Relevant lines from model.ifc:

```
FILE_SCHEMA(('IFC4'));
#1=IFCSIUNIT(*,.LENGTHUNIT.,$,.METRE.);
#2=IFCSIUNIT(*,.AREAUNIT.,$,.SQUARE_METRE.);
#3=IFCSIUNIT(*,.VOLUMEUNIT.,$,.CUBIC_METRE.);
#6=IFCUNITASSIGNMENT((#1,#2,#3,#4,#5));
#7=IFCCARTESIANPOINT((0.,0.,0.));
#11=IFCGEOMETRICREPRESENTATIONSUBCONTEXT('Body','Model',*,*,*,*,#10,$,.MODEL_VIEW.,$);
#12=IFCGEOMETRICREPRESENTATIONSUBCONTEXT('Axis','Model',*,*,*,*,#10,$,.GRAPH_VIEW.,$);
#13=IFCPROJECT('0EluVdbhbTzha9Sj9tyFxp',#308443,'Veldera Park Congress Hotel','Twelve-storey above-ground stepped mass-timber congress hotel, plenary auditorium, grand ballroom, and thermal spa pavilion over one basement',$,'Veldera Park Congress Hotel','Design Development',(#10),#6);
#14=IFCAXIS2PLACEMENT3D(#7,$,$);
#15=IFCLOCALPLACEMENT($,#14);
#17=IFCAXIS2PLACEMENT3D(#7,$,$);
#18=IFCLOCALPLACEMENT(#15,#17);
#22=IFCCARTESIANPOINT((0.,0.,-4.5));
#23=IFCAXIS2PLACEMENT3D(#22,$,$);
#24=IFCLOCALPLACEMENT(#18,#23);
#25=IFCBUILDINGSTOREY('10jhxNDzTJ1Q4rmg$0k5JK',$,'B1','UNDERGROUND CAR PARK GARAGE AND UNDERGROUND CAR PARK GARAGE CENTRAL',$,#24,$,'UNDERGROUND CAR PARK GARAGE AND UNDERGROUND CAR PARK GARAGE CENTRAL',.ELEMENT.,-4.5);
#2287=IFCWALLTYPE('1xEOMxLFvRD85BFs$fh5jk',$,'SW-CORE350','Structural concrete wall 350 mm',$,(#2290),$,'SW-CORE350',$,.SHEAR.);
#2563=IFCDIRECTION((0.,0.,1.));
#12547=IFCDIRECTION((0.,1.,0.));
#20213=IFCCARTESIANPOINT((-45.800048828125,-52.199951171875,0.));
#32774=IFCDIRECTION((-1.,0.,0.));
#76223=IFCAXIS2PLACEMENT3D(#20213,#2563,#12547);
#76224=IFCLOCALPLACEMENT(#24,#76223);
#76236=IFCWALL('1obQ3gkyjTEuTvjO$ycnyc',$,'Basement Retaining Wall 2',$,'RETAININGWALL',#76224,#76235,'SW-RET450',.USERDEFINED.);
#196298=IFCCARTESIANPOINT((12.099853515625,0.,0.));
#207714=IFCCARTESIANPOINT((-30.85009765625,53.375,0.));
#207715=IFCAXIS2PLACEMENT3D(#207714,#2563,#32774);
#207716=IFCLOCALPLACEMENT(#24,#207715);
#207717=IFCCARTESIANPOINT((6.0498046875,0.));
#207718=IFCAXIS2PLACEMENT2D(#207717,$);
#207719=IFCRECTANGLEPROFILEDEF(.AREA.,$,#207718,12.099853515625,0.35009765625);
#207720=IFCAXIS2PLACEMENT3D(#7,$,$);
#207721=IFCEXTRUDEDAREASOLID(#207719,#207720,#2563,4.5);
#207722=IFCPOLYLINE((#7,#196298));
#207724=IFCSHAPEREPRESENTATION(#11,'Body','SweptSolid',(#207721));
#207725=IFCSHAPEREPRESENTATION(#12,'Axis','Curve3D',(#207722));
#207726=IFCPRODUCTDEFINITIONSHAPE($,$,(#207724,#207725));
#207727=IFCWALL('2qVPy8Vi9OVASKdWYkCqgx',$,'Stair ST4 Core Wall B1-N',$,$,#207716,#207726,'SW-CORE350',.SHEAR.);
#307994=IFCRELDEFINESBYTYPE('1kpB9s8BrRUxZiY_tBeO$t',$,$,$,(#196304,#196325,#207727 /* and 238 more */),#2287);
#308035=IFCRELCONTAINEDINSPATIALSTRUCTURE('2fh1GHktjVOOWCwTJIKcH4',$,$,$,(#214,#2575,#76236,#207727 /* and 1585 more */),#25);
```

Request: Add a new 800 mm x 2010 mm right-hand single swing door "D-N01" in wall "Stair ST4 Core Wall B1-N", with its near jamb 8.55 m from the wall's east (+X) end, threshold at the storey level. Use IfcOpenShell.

```python
import numpy as np
import ifcopenshell
import ifcopenshell.api.feature
import ifcopenshell.api.geometry
import ifcopenshell.api.root
import ifcopenshell.api.spatial
import ifcopenshell.geom
import ifcopenshell.util.element
import ifcopenshell.util.placement
import ifcopenshell.util.representation
import ifcopenshell.util.shape
import ifcopenshell.util.unit

model = ifcopenshell.open("model.ifc")
unit_scale = ifcopenshell.util.unit.calculate_unit_scale(model)
settings = ifcopenshell.geom.settings()


def volume(element):
    """Net volume in cubic metres, openings subtracted."""
    shape = ifcopenshell.geom.create_shape(settings, element)
    return ifcopenshell.util.shape.get_volume(shape.geometry)


wall = model.by_guid("2qVPy8Vi9OVASKdWYkCqgx")
storey = ifcopenshell.util.element.get_container(wall, ifc_class="IfcBuildingStorey")
context = ifcopenshell.util.representation.get_context(model, "Model", "Body", "MODEL_VIEW")
before = volume(wall)

width, height, from_end, sill = 0.8, 2.01, 8.55, 0.0  # metres

# The wall runs along its own X axis, and the end named is its -X end.
wall_shape = ifcopenshell.geom.create_shape(settings, wall)
x, y, z = ifcopenshell.util.shape.get_vertices(wall_shape.geometry).T
start = x.min() + from_end
face, thickness = float(y.min()), float(y.max() - y.min())
wall_matrix = ifcopenshell.util.placement.get_local_placement(wall.ObjectPlacement)
level = ifcopenshell.util.placement.get_local_placement(storey.ObjectPlacement)[2, 3]


def in_wall(x, y):
    """Placement at x, y metres in the wall's axes, at sill height."""
    matrix = wall_matrix.copy()
    matrix[:, 3] = wall_matrix @ np.array([x / unit_scale, y / unit_scale, 0.0, 1.0])
    matrix[2, 3] = level + sill / unit_scale
    return matrix


# Opening: a box that overshoots both wall faces by 50 mm.
opening = ifcopenshell.api.root.create_entity(model, ifc_class="IfcOpeningElement", predefined_type="OPENING")
box = ifcopenshell.api.geometry.add_wall_representation(
    model, context=context, length=width, height=height, thickness=thickness + 0.1
)
ifcopenshell.api.geometry.assign_representation(model, product=opening, representation=box)
ifcopenshell.api.geometry.edit_object_placement(model, product=opening, matrix=in_wall(start, face - 0.05), is_si=False)
ifcopenshell.api.feature.add_feature(model, feature=opening, element=wall)

door = ifcopenshell.api.root.create_entity(model, ifc_class="IfcDoor", name="D-N01", predefined_type="DOOR")
door.OverallWidth, door.OverallHeight = width / unit_scale, height / unit_scale
door.OperationType = "SINGLE_SWING_RIGHT"
body = ifcopenshell.api.geometry.add_door_representation(
    model,
    context=context,
    overall_width=door.OverallWidth,
    overall_height=door.OverallHeight,
    operation_type="SINGLE_SWING_RIGHT",
    lining_properties={"LiningDepth": thickness / unit_scale, "ThresholdDepth": thickness / unit_scale},
)
ifcopenshell.api.geometry.assign_representation(model, product=door, representation=body)
ifcopenshell.api.spatial.assign_container(model, products=[door], relating_structure=storey)
ifcopenshell.api.feature.add_filling(model, opening=opening, element=door)

# The lining spans the wall, so the door starts at the wall face.
ifcopenshell.api.geometry.edit_object_placement(model, product=door, matrix=in_wall(start, face), is_si=False)

after = volume(wall)

print(f"wall volume {before:.3f} -> {after:.3f} m3")

model.write("model_updated.ifc")
```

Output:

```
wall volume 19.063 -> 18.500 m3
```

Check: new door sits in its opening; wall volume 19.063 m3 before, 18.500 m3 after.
